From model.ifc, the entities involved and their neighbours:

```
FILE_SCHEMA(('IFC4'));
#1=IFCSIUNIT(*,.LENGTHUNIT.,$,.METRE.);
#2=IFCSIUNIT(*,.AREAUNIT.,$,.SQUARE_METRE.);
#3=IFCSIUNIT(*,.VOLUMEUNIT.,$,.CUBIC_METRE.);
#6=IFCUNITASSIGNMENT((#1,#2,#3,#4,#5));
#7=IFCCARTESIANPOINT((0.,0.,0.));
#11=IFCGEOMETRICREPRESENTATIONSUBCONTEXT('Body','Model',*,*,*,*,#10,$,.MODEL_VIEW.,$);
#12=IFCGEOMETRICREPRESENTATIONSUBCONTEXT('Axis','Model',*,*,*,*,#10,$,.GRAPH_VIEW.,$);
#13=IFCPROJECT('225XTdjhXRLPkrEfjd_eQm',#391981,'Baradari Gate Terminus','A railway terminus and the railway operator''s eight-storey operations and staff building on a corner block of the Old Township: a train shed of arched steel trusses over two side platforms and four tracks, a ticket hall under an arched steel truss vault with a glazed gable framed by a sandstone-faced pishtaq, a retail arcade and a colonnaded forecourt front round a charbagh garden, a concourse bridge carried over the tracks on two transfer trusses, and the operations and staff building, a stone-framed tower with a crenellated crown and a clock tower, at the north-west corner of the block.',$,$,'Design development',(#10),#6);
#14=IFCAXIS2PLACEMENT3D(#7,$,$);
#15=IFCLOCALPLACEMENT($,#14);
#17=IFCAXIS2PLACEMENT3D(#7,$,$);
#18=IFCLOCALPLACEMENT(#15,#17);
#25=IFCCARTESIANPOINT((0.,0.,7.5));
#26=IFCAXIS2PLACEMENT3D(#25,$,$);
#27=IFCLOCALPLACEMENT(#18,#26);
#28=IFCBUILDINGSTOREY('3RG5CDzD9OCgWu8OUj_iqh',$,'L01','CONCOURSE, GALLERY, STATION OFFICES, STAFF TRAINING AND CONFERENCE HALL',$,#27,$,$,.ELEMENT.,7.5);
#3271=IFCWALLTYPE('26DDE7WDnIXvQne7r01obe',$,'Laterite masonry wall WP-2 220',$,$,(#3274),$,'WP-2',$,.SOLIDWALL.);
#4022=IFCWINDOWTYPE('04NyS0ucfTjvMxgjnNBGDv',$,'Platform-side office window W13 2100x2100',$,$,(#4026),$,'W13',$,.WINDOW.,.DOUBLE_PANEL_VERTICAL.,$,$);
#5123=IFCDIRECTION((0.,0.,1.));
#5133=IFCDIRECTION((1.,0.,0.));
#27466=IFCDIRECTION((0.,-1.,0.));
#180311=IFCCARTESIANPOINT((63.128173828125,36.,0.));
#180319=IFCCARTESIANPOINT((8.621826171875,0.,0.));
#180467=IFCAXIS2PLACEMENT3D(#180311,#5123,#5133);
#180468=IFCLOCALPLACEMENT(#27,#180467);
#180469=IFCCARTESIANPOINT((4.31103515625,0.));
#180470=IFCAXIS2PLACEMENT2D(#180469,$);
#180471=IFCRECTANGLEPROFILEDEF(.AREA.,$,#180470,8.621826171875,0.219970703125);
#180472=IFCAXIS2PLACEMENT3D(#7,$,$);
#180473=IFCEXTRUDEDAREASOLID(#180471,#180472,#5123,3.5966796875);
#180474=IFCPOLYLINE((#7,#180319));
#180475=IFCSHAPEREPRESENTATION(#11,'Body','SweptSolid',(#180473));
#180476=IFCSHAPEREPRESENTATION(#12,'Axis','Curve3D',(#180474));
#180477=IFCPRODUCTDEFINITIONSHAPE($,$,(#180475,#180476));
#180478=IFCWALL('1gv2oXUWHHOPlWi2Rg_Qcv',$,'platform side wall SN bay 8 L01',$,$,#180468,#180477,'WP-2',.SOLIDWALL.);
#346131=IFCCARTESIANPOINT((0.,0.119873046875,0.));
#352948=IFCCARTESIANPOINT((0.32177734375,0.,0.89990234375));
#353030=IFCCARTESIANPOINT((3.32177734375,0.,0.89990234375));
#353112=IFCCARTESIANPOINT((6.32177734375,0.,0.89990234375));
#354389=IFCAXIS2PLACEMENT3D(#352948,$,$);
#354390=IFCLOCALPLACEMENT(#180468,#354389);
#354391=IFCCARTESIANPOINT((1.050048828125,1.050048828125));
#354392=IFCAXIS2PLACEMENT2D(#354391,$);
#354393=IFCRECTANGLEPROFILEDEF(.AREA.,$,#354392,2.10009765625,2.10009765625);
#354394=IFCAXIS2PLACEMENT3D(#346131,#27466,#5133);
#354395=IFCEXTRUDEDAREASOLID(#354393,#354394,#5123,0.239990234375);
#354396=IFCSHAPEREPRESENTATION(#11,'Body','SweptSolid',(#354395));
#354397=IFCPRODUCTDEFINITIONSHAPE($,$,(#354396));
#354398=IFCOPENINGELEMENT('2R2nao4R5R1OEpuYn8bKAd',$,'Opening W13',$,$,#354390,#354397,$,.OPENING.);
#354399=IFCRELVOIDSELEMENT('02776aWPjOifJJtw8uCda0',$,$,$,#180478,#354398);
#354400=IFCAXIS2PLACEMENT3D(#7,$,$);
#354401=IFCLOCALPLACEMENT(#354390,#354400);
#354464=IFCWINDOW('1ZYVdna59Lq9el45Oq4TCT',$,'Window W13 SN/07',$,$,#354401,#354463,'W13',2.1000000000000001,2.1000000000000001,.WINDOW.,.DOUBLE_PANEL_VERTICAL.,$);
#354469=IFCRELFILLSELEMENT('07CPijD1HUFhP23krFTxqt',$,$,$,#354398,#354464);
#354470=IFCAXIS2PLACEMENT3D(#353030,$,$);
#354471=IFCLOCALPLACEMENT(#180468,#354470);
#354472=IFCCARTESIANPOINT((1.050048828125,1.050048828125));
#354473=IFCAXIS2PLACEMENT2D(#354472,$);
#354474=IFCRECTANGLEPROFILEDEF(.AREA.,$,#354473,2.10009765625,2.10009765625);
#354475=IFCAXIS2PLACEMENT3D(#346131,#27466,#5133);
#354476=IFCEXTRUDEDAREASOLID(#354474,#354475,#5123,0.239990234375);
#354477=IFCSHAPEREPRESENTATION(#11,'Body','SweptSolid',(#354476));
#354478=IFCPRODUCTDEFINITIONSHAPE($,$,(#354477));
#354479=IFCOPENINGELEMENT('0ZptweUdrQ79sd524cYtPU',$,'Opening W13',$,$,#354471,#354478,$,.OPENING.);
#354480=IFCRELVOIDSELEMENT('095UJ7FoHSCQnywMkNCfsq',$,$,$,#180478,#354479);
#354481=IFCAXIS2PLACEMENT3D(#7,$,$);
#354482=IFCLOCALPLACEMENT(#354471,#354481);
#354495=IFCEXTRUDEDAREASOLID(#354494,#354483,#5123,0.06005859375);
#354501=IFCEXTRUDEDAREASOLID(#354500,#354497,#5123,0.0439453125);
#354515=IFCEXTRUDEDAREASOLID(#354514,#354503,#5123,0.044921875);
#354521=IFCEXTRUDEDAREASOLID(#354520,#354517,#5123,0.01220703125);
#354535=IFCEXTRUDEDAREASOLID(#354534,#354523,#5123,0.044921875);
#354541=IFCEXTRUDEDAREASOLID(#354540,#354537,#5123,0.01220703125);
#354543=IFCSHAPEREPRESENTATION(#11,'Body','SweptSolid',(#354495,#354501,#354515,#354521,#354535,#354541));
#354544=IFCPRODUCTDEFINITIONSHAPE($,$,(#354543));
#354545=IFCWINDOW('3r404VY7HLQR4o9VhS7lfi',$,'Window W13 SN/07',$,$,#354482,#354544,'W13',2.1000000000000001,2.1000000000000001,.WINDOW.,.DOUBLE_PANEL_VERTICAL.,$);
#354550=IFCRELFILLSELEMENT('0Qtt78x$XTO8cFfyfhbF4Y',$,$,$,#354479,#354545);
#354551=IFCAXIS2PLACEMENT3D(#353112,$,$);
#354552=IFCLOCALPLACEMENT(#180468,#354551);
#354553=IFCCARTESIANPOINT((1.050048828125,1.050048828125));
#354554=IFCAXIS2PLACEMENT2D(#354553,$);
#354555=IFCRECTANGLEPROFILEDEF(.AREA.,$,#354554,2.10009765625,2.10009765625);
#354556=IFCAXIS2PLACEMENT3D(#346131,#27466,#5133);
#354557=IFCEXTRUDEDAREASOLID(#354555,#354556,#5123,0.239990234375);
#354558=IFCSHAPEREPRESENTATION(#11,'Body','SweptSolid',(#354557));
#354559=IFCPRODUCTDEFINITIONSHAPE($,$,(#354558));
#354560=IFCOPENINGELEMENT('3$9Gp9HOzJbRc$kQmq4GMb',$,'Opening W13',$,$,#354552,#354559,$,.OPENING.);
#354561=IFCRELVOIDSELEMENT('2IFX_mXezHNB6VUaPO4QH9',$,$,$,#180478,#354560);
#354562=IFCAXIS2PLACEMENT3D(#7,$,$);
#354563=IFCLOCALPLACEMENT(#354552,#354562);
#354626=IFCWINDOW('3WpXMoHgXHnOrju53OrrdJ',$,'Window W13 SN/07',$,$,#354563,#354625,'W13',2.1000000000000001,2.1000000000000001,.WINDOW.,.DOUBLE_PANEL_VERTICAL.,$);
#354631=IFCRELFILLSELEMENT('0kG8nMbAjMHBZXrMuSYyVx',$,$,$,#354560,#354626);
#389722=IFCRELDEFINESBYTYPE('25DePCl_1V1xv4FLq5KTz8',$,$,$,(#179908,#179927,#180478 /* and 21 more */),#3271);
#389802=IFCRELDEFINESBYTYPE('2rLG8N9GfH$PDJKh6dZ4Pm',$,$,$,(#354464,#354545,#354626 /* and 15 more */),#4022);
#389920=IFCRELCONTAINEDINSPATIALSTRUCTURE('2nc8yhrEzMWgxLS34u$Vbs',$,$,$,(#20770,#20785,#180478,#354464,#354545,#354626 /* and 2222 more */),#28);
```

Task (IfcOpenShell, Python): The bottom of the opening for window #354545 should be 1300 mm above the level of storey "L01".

```python
import numpy as np
import ifcopenshell
import ifcopenshell.api.geometry
import ifcopenshell.geom
import ifcopenshell.util.element
import ifcopenshell.util.placement
import ifcopenshell.util.shape
import ifcopenshell.util.unit

model = ifcopenshell.open("model.ifc")
unit_scale = ifcopenshell.util.unit.calculate_unit_scale(model)

window = model.by_guid("3r404VY7HLQR4o9VhS7lfi")
opening = window.FillsVoids[0].RelatingOpeningElement
storey = ifcopenshell.util.element.get_container(window, ifc_class="IfcBuildingStorey")
level = ifcopenshell.util.placement.get_local_placement(storey.ObjectPlacement)[2, 3]

# The opening's origin need not be at the sill, so measure its lowest point.
shape = ifcopenshell.geom.create_shape(ifcopenshell.geom.settings(), opening)
bottom = ifcopenshell.util.shape.get_shape_bottom_elevation(shape, shape.geometry) / unit_scale
dz = level + 1.3 / unit_scale - bottom

shift = np.array([0.0, 0.0, dz])
# The window is placed relative to its opening, so it follows when the opening moves.
matrix = ifcopenshell.util.placement.get_local_placement(opening.ObjectPlacement)
matrix[:3, 3] += shift
ifcopenshell.api.geometry.edit_object_placement(
    model, product=opening, matrix=matrix, is_si=False, should_transform_children=True
)

print(f"moved by {dz * unit_scale:+.3f} m")

model.write("model_edited.ifc")
```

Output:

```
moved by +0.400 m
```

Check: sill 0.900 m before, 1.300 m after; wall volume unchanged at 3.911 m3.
